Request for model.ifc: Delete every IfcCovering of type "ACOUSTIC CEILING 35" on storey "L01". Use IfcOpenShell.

First a look at what the model holds.

```python
import ifcopenshell
import ifcopenshell.util.element

model = ifcopenshell.open("model.ifc")
print(model.schema)
storey = next(s for s in model.by_type("IfcBuildingStorey") if s.Name == "L01")
coverings = [e for e in ifcopenshell.util.element.get_decomposition(storey) if e.is_a("IfcCovering")]
seen = {}
for e in coverings:
    element_type = ifcopenshell.util.element.get_type(e)
    name = element_type.Name if element_type not in (None, e) else None
    seen[name] = seen.get(name, 0) + 1
for name, count in sorted(seen.items(), key=str):
    print(count, "x", name)
```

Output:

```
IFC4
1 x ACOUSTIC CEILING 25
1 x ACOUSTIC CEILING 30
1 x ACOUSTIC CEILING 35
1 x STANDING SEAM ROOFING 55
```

```python
import ifcopenshell
import ifcopenshell.api.root
import ifcopenshell.util.element

model = ifcopenshell.open("model.ifc")

storey = next(s for s in model.by_type("IfcBuildingStorey") if s.Name == "L01")
coverings = [e for e in ifcopenshell.util.element.get_decomposition(storey) if e.is_a("IfcCovering")]
targets = [e for e in coverings if (t := ifcopenshell.util.element.get_type(e)) not in (None, e) and t.Name == "ACOUSTIC CEILING 35"]

for e in targets:
    ifcopenshell.api.root.remove_product(model, product=e)
print(len(targets), "removed")

model.write("model_updated.ifc")
```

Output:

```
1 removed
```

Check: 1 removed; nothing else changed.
